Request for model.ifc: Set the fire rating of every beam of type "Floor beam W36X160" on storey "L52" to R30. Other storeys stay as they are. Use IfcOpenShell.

First a look at what the model holds.

```python
import ifcopenshell
import ifcopenshell.util.element

model = ifcopenshell.open("model.ifc")
print(model.schema)
storey = next(s for s in model.by_type("IfcBuildingStorey") if s.Name == "L52")
beams = [e for e in ifcopenshell.util.element.get_decomposition(storey) if e.is_a("IfcBeam")]
seen = {}
for e in beams:
    element_type = ifcopenshell.util.element.get_type(e)
    key = (element_type.Name if element_type != e and element_type else None, ifcopenshell.util.element.get_pset(e, "Pset_BeamCommon", "FireRating"))
    seen[key] = seen.get(key, 0) + 1
for (name, value), count in sorted(seen.items(), key=str):
    print(count, "x", name, "|", value)
```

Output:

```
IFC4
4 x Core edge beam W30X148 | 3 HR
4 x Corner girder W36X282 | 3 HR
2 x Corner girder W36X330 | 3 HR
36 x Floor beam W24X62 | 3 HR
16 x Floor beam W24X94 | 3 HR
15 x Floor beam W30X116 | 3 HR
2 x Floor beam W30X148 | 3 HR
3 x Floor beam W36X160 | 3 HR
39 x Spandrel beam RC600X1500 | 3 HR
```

```python
import ifcopenshell
import ifcopenshell.api.pset
import ifcopenshell.util.element

model = ifcopenshell.open("model.ifc")

storey = next(s for s in model.by_type("IfcBuildingStorey") if s.Name == "L52")
beams = [e for e in ifcopenshell.util.element.get_decomposition(storey) if e.is_a("IfcBeam")]

count = 0
for e in beams:
    element_type = ifcopenshell.util.element.get_type(e)
    if element_type in (None, e) or element_type.Name != "Floor beam W36X160":
        continue
    found = ifcopenshell.util.element.get_pset(e, "Pset_BeamCommon", should_inherit=False)
    if found:
        pset = model.by_id(found["id"])
        if len(ifcopenshell.util.element.get_elements_by_pset(pset)) > 1:
            pset = ifcopenshell.api.pset.unshare_pset(model, products=[e], pset=pset)[0]
    else:
        pset = ifcopenshell.api.pset.add_pset(model, product=e, name="Pset_BeamCommon")
    ifcopenshell.api.pset.edit_pset(model, pset=pset, properties={"FireRating": "R30"})
    count += 1

print(count, "beams updated")

model.write("model_updated.ifc")
```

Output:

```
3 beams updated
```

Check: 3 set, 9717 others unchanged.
